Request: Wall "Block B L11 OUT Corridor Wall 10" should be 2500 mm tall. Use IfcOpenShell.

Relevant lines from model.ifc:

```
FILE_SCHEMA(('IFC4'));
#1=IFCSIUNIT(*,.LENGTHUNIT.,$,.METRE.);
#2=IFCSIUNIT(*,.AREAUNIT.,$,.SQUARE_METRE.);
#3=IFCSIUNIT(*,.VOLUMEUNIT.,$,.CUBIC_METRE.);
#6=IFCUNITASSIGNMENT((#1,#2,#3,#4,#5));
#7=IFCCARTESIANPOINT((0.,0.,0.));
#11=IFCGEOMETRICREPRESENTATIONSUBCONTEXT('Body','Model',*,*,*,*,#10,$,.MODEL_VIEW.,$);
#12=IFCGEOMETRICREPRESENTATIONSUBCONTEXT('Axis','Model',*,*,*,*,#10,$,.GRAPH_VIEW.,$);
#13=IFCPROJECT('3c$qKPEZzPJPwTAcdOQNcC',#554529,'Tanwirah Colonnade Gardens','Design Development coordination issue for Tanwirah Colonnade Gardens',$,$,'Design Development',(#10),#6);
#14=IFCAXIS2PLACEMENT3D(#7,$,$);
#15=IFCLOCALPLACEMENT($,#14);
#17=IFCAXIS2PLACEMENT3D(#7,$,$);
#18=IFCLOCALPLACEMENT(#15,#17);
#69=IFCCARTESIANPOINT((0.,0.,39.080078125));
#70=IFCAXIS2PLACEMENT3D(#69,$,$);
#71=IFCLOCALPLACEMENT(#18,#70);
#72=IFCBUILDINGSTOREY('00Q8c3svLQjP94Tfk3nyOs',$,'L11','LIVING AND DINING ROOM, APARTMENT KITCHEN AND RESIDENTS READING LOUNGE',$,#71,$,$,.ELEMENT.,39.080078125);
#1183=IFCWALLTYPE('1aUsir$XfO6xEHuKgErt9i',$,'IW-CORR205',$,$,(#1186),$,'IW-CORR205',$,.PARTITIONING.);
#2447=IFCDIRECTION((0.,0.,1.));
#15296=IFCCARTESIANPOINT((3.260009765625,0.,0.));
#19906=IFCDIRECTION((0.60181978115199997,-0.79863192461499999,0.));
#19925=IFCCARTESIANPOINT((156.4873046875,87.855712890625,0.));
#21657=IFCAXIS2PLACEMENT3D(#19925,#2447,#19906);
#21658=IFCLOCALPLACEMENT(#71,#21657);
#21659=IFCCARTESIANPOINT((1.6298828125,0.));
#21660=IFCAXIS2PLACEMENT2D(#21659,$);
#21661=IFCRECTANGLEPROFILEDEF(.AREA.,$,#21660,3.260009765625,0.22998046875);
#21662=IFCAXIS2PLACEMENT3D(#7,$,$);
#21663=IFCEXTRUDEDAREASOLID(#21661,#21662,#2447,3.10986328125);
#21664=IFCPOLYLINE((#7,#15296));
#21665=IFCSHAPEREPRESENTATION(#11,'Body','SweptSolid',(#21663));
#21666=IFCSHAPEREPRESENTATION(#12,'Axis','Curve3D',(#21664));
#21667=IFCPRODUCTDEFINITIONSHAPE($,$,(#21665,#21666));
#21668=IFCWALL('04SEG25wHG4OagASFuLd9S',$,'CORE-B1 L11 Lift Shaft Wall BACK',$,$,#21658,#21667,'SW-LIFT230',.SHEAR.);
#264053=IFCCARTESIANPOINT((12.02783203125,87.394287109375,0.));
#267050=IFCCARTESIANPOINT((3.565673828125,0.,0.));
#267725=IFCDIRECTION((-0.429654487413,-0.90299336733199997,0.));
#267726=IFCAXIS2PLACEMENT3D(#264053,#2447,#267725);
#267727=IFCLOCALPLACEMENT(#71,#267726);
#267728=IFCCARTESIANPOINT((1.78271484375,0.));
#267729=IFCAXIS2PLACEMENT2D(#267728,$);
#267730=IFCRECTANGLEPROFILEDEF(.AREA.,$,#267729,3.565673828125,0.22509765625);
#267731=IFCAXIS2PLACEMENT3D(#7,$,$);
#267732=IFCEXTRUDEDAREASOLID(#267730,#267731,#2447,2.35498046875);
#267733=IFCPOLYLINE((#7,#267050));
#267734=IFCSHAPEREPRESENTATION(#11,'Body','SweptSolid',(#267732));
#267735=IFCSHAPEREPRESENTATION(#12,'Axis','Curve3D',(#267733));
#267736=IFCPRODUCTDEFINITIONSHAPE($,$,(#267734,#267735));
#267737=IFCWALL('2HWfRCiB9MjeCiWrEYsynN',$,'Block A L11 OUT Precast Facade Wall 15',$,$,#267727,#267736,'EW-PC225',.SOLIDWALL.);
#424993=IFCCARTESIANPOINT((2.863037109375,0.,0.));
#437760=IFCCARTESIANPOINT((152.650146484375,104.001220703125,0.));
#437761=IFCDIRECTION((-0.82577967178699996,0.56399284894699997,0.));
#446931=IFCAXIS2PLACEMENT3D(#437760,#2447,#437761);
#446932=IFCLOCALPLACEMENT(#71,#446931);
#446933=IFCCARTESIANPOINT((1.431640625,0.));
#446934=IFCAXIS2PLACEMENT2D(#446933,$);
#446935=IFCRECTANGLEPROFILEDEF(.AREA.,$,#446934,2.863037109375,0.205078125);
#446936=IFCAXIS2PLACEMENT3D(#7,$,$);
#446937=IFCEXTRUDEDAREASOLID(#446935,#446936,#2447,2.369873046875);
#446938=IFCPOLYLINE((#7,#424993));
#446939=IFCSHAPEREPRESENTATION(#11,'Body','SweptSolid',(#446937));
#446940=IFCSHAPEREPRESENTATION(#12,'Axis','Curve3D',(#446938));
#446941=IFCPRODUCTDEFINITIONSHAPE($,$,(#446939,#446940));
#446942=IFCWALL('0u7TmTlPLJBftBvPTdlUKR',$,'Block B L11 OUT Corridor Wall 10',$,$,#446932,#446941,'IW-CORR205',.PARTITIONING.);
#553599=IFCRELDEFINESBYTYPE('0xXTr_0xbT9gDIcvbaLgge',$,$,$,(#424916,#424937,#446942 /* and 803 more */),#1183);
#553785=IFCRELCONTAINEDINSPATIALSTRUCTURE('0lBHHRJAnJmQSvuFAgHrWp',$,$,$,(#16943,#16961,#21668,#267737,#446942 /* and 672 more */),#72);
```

```python
import ifcopenshell
import ifcopenshell.geom
import ifcopenshell.util.representation
import ifcopenshell.util.shape
import ifcopenshell.util.unit

model = ifcopenshell.open("model.ifc")
unit_scale = ifcopenshell.util.unit.calculate_unit_scale(model)
settings = ifcopenshell.geom.settings()


def volume(element):
    """Net volume in cubic metres, openings subtracted."""
    shape = ifcopenshell.geom.create_shape(settings, element)
    return ifcopenshell.util.shape.get_volume(shape.geometry)


wall = model.by_id(446942)
before = volume(wall)

body = ifcopenshell.util.representation.get_representation(wall, "Model", "Body")
solid = body.Items[0]
old_height = solid.Depth
solid.Depth = 2.5 / unit_scale
after = volume(wall)

print(f"height {old_height:g} -> {solid.Depth:g}, volume {before:.3f} -> {after:.3f} m3")

model.write("model-out.ifc")
```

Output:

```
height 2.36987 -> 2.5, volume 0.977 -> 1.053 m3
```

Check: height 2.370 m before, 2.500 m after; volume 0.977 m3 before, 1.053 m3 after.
